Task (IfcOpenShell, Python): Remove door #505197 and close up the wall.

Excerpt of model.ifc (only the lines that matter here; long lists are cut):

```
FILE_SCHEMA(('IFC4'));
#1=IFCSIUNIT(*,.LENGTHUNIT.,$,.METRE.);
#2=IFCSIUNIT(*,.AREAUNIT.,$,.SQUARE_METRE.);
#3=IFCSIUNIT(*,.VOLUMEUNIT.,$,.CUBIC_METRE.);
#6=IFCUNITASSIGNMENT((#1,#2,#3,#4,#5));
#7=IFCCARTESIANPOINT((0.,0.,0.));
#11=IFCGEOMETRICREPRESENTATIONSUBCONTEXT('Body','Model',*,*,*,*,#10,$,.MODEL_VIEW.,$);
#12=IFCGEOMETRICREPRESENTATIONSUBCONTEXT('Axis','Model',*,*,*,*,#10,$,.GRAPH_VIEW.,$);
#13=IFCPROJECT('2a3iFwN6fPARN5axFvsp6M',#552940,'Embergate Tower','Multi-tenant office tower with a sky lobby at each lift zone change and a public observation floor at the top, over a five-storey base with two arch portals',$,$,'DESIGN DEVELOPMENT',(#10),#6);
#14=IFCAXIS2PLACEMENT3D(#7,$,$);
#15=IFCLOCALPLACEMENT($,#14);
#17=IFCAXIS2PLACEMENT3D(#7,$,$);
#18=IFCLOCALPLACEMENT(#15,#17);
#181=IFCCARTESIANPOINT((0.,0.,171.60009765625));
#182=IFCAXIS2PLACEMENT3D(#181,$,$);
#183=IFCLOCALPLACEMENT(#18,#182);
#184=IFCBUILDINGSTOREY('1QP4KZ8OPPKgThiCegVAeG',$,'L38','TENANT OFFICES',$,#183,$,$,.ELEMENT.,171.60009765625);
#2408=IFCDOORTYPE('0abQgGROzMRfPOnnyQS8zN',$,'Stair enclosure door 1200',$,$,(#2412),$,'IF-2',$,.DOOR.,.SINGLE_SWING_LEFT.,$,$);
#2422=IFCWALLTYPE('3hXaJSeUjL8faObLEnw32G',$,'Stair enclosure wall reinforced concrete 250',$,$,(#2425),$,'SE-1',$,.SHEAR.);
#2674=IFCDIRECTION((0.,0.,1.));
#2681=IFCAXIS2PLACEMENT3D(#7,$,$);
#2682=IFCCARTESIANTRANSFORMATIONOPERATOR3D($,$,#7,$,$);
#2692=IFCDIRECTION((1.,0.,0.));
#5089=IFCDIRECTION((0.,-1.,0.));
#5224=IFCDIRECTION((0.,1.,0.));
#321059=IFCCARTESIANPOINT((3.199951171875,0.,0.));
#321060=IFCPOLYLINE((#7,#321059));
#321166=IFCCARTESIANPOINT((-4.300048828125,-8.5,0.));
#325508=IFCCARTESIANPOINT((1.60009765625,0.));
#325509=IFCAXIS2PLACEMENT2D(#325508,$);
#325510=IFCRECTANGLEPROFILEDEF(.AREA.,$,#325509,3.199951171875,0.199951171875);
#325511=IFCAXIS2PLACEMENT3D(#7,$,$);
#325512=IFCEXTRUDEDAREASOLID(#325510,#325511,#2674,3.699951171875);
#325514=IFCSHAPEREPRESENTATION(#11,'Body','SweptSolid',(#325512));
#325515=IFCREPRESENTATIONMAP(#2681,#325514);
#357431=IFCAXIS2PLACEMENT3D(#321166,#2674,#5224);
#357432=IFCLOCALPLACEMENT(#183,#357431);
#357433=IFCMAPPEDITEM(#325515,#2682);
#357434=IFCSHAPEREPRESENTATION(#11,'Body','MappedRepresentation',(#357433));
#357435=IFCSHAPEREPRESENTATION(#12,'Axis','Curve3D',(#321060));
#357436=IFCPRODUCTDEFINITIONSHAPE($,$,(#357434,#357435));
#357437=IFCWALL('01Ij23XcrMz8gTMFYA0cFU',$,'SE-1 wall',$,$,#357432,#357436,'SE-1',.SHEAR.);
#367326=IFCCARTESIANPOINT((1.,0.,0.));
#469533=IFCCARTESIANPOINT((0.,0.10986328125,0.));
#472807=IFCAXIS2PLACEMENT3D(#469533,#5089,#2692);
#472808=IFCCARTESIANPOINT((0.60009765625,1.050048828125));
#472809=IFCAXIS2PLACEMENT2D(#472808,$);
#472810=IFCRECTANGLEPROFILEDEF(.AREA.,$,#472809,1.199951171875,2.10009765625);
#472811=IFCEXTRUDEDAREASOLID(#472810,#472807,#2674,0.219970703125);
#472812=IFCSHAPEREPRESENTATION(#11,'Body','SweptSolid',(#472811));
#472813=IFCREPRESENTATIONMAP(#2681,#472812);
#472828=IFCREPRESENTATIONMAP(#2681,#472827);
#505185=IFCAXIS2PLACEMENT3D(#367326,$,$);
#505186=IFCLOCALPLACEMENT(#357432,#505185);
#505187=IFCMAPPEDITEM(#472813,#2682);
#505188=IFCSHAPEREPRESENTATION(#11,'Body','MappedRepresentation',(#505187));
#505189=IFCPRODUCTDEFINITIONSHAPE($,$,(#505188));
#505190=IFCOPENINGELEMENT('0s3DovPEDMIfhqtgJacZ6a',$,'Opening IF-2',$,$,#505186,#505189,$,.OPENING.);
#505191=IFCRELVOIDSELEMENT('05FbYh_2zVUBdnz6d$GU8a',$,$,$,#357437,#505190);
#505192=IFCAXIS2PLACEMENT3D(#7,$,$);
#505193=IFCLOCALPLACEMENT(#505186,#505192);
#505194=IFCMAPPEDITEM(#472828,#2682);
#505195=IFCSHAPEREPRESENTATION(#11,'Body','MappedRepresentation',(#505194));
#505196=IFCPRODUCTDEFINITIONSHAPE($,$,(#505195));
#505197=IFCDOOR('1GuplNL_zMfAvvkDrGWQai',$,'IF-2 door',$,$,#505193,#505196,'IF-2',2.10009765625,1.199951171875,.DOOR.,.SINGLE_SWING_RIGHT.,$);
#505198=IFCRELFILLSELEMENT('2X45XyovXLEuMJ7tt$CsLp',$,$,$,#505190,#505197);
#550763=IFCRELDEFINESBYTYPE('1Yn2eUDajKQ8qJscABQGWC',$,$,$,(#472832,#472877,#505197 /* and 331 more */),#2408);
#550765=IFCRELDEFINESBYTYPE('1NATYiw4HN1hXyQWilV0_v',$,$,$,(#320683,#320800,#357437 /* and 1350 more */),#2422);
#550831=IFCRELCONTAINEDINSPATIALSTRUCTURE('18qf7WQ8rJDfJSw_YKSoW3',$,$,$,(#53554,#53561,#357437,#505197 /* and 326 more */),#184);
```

```python
import ifcopenshell
import ifcopenshell.api.feature
import ifcopenshell.api.root
import ifcopenshell.geom
import ifcopenshell.util.shape

model = ifcopenshell.open("model.ifc")
settings = ifcopenshell.geom.settings()


def volume(element):
    """Net volume in cubic metres, openings subtracted."""
    shape = ifcopenshell.geom.create_shape(settings, element)
    return ifcopenshell.util.shape.get_volume(shape.geometry)


door = model.by_guid("1GuplNL_zMfAvvkDrGWQai")
opening = door.FillsVoids[0].RelatingOpeningElement
wall = opening.VoidsElements[0].RelatingBuildingElement
before = volume(wall)

ifcopenshell.api.root.remove_product(model, product=door)
ifcopenshell.api.feature.remove_feature(model, feature=opening)

after = volume(wall)

print(f"wall volume {before:.3f} -> {after:.3f} m3")

model.write("model_edited.ifc")
```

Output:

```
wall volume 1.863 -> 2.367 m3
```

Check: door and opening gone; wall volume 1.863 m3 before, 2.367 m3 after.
